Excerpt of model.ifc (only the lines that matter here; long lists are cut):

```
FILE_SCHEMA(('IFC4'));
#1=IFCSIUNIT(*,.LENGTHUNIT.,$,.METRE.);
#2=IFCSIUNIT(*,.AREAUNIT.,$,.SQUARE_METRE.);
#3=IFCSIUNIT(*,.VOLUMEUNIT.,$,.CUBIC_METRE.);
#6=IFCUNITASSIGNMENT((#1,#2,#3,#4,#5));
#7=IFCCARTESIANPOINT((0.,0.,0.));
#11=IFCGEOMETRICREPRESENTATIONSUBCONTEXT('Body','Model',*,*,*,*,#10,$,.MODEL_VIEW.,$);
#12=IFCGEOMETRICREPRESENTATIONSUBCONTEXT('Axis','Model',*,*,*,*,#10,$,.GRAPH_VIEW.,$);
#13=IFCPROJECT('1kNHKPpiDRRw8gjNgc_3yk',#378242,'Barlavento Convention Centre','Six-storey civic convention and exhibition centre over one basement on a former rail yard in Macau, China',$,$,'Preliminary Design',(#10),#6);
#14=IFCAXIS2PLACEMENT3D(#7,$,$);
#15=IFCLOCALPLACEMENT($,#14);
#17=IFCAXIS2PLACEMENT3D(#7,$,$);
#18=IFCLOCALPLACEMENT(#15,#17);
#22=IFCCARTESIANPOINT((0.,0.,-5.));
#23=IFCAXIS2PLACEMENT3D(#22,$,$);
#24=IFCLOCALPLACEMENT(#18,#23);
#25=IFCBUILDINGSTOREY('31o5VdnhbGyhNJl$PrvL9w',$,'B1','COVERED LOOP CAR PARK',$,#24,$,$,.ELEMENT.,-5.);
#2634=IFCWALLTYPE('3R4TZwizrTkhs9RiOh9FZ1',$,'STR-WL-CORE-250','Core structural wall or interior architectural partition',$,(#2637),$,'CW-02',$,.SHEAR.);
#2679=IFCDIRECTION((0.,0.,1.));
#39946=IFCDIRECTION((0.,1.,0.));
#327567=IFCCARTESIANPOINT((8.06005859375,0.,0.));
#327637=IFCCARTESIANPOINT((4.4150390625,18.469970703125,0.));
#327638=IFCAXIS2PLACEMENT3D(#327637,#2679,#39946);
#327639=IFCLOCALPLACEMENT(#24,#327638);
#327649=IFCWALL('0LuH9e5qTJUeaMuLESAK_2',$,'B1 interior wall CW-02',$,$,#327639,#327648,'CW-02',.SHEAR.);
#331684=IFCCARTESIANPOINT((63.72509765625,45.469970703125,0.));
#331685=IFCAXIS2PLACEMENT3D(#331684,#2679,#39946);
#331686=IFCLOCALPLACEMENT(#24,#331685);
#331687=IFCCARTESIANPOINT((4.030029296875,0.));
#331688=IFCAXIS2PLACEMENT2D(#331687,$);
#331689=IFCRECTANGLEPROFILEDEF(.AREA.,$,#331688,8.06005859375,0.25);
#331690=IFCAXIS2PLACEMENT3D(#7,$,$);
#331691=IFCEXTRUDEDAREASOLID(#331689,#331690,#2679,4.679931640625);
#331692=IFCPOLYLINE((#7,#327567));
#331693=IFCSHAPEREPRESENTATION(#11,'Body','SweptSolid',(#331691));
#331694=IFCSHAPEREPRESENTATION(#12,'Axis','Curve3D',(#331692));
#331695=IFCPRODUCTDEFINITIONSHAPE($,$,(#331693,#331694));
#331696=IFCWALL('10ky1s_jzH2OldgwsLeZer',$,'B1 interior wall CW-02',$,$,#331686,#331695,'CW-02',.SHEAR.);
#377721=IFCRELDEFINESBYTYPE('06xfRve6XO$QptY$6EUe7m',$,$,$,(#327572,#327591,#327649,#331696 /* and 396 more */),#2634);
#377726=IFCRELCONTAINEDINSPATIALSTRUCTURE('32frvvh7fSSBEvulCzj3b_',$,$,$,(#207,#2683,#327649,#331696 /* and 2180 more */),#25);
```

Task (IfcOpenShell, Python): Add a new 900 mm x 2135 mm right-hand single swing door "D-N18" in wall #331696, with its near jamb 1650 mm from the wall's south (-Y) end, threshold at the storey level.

```python
import numpy as np
import ifcopenshell
import ifcopenshell.api.feature
import ifcopenshell.api.geometry
import ifcopenshell.api.root
import ifcopenshell.api.spatial
import ifcopenshell.geom
import ifcopenshell.util.element
import ifcopenshell.util.placement
import ifcopenshell.util.representation
import ifcopenshell.util.shape
import ifcopenshell.util.unit

model = ifcopenshell.open("model.ifc")
unit_scale = ifcopenshell.util.unit.calculate_unit_scale(model)
settings = ifcopenshell.geom.settings()


def volume(element):
    """Net volume in cubic metres, openings subtracted."""
    shape = ifcopenshell.geom.create_shape(settings, element)
    return ifcopenshell.util.shape.get_volume(shape.geometry)


wall = model.by_id(331696)
storey = ifcopenshell.util.element.get_container(wall, ifc_class="IfcBuildingStorey")
context = ifcopenshell.util.representation.get_context(model, "Model", "Body", "MODEL_VIEW")
before = volume(wall)

width, height, from_end, sill = 0.9, 2.135, 1.65, 0.0  # metres

# The wall runs along its own X axis, and the end named is its -X end.
wall_shape = ifcopenshell.geom.create_shape(settings, wall)
x, y, z = ifcopenshell.util.shape.get_vertices(wall_shape.geometry).T
start = x.min() + from_end
face, thickness = float(y.min()), float(y.max() - y.min())
wall_matrix = ifcopenshell.util.placement.get_local_placement(wall.ObjectPlacement)
level = ifcopenshell.util.placement.get_local_placement(storey.ObjectPlacement)[2, 3]


def in_wall(x, y):
    """Placement at x, y metres in the wall's axes, at sill height."""
    matrix = wall_matrix.copy()
    matrix[:, 3] = wall_matrix @ np.array([x / unit_scale, y / unit_scale, 0.0, 1.0])
    matrix[2, 3] = level + sill / unit_scale
    return matrix


# Opening: a box that overshoots both wall faces by 50 mm.
opening = ifcopenshell.api.root.create_entity(model, ifc_class="IfcOpeningElement", predefined_type="OPENING")
box = ifcopenshell.api.geometry.add_wall_representation(
    model, context=context, length=width, height=height, thickness=thickness + 0.1
)
ifcopenshell.api.geometry.assign_representation(model, product=opening, representation=box)
ifcopenshell.api.geometry.edit_object_placement(model, product=opening, matrix=in_wall(start, face - 0.05), is_si=False)
ifcopenshell.api.feature.add_feature(model, feature=opening, element=wall)

door = ifcopenshell.api.root.create_entity(model, ifc_class="IfcDoor", name="D-N18", predefined_type="DOOR")
door.OverallWidth, door.OverallHeight = width / unit_scale, height / unit_scale
door.OperationType = "SINGLE_SWING_RIGHT"
body = ifcopenshell.api.geometry.add_door_representation(
    model,
    context=context,
    overall_width=door.OverallWidth,
    overall_height=door.OverallHeight,
    operation_type="SINGLE_SWING_RIGHT",
    lining_properties={"LiningDepth": thickness / unit_scale, "ThresholdDepth": thickness / unit_scale},
)
ifcopenshell.api.geometry.assign_representation(model, product=door, representation=body)
ifcopenshell.api.spatial.assign_container(model, products=[door], relating_structure=storey)
ifcopenshell.api.feature.add_filling(model, opening=opening, element=door)

# The lining spans the wall, so the door starts at the wall face.
ifcopenshell.api.geometry.edit_object_placement(model, product=door, matrix=in_wall(start, face), is_si=False)

after = volume(wall)

print(f"wall volume {before:.3f} -> {after:.3f} m3")

model.write("model_rev.ifc")
```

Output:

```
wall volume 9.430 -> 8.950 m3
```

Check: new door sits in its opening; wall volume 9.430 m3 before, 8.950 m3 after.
